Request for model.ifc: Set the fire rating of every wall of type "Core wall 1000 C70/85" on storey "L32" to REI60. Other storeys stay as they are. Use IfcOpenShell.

First a look at what the model holds.

```python
import ifcopenshell
import ifcopenshell.util.element

model = ifcopenshell.open("model.ifc")
print(model.schema)
storey = next(s for s in model.by_type("IfcBuildingStorey") if s.Name == "L32")
walls = [e for e in ifcopenshell.util.element.get_decomposition(storey) if e.is_a("IfcWall")]
seen = {}
for e in walls:
    element_type = ifcopenshell.util.element.get_type(e)
    key = (element_type.Name if element_type != e and element_type else None, ifcopenshell.util.element.get_pset(e, "Pset_WallCommon", "FireRating"))
    seen[key] = seen.get(key, 0) + 1
for (name, value), count in sorted(seen.items(), key=str):
    print(count, "x", name, "|", value)
```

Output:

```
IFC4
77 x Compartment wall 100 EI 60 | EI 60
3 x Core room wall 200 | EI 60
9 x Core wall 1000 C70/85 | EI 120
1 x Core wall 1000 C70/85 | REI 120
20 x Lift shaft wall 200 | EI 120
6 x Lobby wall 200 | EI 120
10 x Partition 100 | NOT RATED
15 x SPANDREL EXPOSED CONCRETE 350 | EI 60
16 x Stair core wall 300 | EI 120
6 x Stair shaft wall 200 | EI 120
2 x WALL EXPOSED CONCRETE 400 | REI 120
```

```python
import ifcopenshell
import ifcopenshell.api.pset
import ifcopenshell.util.element

model = ifcopenshell.open("model.ifc")

storey = next(s for s in model.by_type("IfcBuildingStorey") if s.Name == "L32")
walls = [e for e in ifcopenshell.util.element.get_decomposition(storey) if e.is_a("IfcWall")]

count = 0
for e in walls:
    element_type = ifcopenshell.util.element.get_type(e)
    if element_type in (None, e) or element_type.Name != "Core wall 1000 C70/85":
        continue
    found = ifcopenshell.util.element.get_pset(e, "Pset_WallCommon", should_inherit=False)
    if found:
        pset = model.by_id(found["id"])
        if len(ifcopenshell.util.element.get_elements_by_pset(pset)) > 1:
            pset = ifcopenshell.api.pset.unshare_pset(model, products=[e], pset=pset)[0]
    else:
        pset = ifcopenshell.api.pset.add_pset(model, product=e, name="Pset_WallCommon")
    ifcopenshell.api.pset.edit_pset(model, pset=pset, properties={"FireRating": "REI60"})
    count += 1

print(count, "walls updated")

model.write("model-out.ifc")
```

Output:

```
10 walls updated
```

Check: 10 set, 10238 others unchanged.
